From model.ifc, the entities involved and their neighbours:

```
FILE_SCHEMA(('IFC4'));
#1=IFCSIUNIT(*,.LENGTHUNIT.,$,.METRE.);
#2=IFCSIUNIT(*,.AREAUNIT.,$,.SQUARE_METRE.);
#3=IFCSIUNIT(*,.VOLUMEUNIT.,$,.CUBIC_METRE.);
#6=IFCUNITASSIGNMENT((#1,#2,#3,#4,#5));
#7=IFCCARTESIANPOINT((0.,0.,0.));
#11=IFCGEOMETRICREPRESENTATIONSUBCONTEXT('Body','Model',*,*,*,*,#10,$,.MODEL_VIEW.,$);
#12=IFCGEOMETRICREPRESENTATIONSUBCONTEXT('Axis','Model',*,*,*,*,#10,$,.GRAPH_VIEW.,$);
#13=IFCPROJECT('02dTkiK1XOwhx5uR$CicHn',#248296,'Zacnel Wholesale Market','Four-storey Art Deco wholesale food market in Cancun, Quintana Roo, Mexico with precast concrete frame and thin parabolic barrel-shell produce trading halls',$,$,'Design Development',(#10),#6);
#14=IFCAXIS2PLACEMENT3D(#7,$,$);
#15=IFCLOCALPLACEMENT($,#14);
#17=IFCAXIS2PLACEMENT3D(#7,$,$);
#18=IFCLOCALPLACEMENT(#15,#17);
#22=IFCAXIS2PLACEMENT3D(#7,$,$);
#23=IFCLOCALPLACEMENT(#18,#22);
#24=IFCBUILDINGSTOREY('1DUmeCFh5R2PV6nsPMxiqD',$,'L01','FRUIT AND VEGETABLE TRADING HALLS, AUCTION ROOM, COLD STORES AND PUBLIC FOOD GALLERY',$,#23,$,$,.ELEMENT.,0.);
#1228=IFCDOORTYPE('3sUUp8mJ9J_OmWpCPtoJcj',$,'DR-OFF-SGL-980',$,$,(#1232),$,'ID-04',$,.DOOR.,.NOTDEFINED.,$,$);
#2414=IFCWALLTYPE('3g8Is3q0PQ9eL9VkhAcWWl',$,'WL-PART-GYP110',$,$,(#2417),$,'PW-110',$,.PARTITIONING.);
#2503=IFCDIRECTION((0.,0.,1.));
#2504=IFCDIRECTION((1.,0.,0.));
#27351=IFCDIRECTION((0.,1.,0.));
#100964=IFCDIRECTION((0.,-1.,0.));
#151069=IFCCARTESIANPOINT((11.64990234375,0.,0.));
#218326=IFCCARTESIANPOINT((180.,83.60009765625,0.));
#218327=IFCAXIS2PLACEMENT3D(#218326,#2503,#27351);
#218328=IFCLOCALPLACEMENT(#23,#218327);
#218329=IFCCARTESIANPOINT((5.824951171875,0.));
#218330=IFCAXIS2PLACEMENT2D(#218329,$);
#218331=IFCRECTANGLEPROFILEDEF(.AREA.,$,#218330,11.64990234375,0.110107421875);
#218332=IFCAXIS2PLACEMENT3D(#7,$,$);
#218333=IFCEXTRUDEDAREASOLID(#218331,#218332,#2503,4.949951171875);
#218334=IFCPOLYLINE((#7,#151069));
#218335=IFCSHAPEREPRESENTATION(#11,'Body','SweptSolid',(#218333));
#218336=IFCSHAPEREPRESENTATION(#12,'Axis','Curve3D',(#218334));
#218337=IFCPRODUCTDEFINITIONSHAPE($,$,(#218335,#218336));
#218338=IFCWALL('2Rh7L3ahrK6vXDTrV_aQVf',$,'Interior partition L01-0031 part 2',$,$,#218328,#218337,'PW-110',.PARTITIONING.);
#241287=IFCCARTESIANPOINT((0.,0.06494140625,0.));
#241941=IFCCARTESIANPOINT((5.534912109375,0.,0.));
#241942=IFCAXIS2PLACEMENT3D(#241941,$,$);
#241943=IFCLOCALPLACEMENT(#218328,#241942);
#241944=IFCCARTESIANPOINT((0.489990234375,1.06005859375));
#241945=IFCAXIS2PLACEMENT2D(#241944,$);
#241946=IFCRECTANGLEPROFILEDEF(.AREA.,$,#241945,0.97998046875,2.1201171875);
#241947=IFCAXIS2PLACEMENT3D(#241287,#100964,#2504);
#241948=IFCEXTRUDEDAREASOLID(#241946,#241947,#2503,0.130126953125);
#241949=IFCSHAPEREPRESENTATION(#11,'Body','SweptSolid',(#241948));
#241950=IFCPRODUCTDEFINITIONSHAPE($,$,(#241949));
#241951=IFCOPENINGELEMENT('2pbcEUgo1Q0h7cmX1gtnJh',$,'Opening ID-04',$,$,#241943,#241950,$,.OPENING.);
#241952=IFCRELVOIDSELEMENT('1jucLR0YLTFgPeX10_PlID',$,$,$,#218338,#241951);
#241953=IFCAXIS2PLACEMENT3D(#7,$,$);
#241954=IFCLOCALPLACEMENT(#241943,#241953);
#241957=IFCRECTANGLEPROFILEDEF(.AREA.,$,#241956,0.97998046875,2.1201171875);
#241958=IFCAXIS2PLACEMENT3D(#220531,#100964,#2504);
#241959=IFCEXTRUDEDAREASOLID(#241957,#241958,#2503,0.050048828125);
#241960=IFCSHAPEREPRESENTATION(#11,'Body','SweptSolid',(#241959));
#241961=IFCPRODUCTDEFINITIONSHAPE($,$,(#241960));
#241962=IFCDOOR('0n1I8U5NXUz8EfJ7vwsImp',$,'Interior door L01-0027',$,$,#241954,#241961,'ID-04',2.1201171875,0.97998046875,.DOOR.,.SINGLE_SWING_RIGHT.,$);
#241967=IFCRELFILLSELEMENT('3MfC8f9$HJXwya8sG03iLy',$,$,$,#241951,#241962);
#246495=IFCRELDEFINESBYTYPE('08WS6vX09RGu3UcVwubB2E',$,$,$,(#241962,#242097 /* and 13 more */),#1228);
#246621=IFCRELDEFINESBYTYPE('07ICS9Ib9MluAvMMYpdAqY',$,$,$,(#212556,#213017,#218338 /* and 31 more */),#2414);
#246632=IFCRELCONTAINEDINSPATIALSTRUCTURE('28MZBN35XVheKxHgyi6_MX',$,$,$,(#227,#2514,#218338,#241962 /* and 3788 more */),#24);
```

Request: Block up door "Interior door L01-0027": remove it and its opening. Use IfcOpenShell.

```python
import ifcopenshell
import ifcopenshell.api.feature
import ifcopenshell.api.root
import ifcopenshell.geom
import ifcopenshell.util.shape

model = ifcopenshell.open("model.ifc")
settings = ifcopenshell.geom.settings()


def volume(element):
    """Net volume in cubic metres, openings subtracted."""
    shape = ifcopenshell.geom.create_shape(settings, element)
    return ifcopenshell.util.shape.get_volume(shape.geometry)


door = model.by_guid("0n1I8U5NXUz8EfJ7vwsImp")
opening = door.FillsVoids[0].RelatingOpeningElement
wall = opening.VoidsElements[0].RelatingBuildingElement
before = volume(wall)

ifcopenshell.api.root.remove_product(model, product=door)
ifcopenshell.api.feature.remove_feature(model, feature=opening)

after = volume(wall)

print(f"wall volume {before:.3f} -> {after:.3f} m3")

model.write("model_updated.ifc")
```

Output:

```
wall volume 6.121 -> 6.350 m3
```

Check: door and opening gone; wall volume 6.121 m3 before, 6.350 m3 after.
